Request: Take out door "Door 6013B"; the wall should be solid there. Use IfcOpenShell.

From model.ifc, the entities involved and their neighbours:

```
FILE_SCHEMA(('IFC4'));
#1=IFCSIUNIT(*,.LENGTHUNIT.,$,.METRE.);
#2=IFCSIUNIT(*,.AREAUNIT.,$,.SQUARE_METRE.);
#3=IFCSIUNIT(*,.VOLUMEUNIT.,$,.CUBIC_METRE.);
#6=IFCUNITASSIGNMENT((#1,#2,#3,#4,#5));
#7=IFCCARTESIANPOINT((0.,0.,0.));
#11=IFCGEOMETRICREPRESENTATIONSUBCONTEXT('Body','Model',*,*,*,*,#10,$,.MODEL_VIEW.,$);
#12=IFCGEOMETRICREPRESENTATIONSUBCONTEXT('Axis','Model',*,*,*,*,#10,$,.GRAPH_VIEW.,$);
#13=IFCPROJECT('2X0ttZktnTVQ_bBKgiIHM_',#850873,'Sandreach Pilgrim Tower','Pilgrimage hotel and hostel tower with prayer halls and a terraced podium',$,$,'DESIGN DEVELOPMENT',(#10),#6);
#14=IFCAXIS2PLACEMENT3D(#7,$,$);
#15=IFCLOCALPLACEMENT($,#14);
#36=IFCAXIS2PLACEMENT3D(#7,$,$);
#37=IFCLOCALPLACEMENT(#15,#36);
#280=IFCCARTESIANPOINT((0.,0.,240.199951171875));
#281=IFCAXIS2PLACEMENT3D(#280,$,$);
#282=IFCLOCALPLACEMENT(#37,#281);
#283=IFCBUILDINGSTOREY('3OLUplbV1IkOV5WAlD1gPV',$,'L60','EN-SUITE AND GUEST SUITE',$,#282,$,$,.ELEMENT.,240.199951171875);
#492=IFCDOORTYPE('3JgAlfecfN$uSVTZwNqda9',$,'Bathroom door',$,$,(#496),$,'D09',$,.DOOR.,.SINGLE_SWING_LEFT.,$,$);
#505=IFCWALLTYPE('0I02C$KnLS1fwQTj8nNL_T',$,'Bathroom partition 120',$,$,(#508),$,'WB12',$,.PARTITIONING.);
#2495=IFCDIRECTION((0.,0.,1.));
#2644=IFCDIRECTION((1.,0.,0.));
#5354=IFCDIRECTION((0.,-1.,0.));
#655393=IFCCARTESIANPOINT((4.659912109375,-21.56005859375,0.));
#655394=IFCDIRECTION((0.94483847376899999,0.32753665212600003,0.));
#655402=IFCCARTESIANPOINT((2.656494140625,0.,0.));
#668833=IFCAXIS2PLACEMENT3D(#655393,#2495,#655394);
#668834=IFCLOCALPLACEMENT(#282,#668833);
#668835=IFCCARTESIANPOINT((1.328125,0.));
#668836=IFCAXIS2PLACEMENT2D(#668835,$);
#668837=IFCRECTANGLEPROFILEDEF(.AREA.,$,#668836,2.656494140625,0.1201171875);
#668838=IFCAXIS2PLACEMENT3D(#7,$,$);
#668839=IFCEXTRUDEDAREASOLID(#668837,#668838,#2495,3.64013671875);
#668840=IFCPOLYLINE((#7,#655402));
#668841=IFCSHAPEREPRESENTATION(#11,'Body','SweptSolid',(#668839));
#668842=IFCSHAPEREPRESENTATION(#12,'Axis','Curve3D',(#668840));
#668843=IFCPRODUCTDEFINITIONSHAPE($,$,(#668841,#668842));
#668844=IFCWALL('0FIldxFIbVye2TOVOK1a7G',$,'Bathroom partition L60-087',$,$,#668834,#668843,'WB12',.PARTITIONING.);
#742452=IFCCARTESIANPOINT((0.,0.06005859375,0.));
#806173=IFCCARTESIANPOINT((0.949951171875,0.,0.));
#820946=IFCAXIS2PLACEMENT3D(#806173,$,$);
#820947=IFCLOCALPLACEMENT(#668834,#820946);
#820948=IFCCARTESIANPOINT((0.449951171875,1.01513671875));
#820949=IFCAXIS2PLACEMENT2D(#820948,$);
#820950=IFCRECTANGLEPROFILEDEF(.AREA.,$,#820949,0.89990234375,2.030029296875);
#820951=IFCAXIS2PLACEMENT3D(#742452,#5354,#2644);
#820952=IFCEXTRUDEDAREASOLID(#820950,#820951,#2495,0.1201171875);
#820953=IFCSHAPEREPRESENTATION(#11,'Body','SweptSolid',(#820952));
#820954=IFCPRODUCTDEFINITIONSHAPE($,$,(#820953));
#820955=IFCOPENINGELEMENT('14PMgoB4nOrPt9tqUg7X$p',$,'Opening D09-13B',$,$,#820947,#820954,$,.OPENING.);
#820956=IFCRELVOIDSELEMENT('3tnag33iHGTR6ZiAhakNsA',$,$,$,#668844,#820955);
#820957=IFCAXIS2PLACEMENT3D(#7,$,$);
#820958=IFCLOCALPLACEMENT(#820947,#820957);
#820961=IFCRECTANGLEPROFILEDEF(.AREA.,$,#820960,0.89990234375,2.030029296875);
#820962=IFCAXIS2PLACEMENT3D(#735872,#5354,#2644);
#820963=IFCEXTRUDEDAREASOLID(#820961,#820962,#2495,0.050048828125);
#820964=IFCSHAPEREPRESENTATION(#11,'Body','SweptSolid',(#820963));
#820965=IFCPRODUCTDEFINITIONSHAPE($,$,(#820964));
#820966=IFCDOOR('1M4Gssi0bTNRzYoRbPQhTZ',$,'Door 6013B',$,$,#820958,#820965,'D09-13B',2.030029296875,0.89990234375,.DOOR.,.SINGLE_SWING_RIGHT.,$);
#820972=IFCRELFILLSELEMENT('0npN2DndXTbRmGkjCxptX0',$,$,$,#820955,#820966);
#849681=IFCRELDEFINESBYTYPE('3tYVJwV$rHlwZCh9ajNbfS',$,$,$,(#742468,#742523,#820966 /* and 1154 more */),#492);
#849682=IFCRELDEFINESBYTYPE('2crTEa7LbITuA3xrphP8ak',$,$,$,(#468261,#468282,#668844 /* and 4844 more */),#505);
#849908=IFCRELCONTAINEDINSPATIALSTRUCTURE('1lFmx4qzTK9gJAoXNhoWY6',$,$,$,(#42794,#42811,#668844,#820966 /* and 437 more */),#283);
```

```python
import ifcopenshell
import ifcopenshell.api.feature
import ifcopenshell.api.root
import ifcopenshell.geom
import ifcopenshell.util.shape

model = ifcopenshell.open("model.ifc")
settings = ifcopenshell.geom.settings()


def volume(element):
    """Net volume in cubic metres, openings subtracted."""
    shape = ifcopenshell.geom.create_shape(settings, element)
    return ifcopenshell.util.shape.get_volume(shape.geometry)


door = model.by_guid("1M4Gssi0bTNRzYoRbPQhTZ")
opening = door.FillsVoids[0].RelatingOpeningElement
wall = opening.VoidsElements[0].RelatingBuildingElement
before = volume(wall)

ifcopenshell.api.root.remove_product(model, product=door)
ifcopenshell.api.feature.remove_feature(model, feature=opening)

after = volume(wall)

print(f"wall volume {before:.3f} -> {after:.3f} m3")

model.write("model_rev.ifc")
```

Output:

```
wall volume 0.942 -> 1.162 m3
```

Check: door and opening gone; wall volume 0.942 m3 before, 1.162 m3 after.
